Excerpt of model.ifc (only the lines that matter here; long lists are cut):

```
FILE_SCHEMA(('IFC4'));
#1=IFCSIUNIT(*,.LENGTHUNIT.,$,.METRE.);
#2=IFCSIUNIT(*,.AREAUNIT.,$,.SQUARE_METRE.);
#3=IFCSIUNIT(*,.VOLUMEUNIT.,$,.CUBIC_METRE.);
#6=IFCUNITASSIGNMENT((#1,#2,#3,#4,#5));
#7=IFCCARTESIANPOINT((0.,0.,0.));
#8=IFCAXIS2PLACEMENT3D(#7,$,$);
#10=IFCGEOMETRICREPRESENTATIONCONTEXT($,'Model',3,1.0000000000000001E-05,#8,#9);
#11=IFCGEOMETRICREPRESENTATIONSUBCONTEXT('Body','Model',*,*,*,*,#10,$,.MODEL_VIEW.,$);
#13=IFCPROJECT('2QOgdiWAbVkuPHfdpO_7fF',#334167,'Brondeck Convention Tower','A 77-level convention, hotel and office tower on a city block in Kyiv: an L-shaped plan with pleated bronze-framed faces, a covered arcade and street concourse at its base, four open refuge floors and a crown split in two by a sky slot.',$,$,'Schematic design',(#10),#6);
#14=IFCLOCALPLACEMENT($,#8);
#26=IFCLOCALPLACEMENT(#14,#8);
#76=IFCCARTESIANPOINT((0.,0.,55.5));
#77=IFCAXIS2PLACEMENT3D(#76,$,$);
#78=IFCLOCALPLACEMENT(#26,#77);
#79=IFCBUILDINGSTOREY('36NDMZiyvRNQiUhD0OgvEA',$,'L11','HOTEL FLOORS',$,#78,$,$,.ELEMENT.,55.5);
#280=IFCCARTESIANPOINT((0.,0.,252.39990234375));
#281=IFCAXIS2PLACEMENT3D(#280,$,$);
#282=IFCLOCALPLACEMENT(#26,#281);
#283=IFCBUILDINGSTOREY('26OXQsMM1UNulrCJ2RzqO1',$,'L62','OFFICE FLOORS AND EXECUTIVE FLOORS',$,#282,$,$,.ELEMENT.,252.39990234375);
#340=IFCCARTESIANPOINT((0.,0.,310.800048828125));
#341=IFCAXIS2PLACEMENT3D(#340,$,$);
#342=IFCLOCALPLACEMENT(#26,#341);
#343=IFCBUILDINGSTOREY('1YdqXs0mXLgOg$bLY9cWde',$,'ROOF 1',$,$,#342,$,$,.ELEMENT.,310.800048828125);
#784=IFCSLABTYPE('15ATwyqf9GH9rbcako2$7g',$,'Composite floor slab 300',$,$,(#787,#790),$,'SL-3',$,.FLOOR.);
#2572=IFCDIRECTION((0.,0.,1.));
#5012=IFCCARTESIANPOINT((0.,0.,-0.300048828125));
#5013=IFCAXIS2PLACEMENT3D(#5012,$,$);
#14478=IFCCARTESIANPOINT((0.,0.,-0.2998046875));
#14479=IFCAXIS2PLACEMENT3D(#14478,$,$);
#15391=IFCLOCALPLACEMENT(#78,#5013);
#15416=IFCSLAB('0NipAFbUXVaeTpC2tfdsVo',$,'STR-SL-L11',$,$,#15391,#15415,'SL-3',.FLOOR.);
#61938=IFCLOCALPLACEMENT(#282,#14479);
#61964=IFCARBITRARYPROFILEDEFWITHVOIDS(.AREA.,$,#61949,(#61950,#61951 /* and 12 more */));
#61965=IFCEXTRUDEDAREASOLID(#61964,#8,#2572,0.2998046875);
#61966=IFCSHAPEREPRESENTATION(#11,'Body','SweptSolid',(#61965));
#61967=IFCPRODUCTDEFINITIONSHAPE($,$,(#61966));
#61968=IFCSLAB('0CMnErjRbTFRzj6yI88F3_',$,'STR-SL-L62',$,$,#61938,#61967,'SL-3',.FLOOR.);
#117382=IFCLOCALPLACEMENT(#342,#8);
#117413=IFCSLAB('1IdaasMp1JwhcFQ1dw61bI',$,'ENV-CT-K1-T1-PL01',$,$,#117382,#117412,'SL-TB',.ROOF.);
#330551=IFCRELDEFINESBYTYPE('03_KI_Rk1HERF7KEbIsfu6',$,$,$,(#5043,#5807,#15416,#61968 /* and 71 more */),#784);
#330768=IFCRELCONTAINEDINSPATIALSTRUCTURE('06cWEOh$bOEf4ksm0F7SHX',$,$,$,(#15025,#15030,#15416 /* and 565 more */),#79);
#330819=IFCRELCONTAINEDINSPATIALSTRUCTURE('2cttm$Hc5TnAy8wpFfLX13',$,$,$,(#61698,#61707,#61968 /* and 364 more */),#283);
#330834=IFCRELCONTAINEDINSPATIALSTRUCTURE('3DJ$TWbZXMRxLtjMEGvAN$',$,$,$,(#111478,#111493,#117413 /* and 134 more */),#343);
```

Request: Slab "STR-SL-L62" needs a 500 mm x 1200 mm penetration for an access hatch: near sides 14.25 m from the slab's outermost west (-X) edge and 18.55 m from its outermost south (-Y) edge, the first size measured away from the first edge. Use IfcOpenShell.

```python
import numpy as np
import ifcopenshell
import ifcopenshell.api.feature
import ifcopenshell.api.geometry
import ifcopenshell.api.root
import ifcopenshell.geom
import ifcopenshell.util.placement
import ifcopenshell.util.representation
import ifcopenshell.util.shape
import ifcopenshell.util.unit

model = ifcopenshell.open("model.ifc")
unit_scale = ifcopenshell.util.unit.calculate_unit_scale(model)
settings = ifcopenshell.geom.settings()


def volume(element):
    """Net volume in cubic metres, openings subtracted."""
    shape = ifcopenshell.geom.create_shape(settings, element)
    return ifcopenshell.util.shape.get_volume(shape.geometry)


slab = model.by_guid("0CMnErjRbTFRzj6yI88F3_")
before = volume(slab)

# Extent in the slab's own axes, in metres. The edges named are its -X and -Y sides.
slab_shape = ifcopenshell.geom.create_shape(settings, slab)
vertices = ifcopenshell.util.shape.get_vertices(slab_shape.geometry)
x_min, y_min, bottom = vertices.min(axis=0)
top = vertices[:, 2].max()

opening = ifcopenshell.api.root.create_entity(model, ifc_class="IfcOpeningElement", name="Access hatch opening", predefined_type="OPENING")
context = ifcopenshell.util.representation.get_context(model, "Model", "Body", "MODEL_VIEW")
width, depth = 0.5, 1.2
outline = [(0.0, 0.0), (width, 0.0), (width, depth), (0.0, depth), (0.0, 0.0)]
# Overshoot both faces by 50 mm so the cut is clean.
shape = ifcopenshell.api.geometry.add_slab_representation(
    model, context=context, depth=top - bottom + 0.1, polyline=outline
)
ifcopenshell.api.geometry.assign_representation(model, product=opening, representation=shape)

matrix = ifcopenshell.util.placement.get_local_placement(slab.ObjectPlacement)
matrix[:, 3] = matrix @ np.append(np.array([x_min + 14.25, y_min + 18.55, bottom - 0.05]) / unit_scale, 1.0)
ifcopenshell.api.geometry.edit_object_placement(model, product=opening, matrix=matrix, is_si=False)
ifcopenshell.api.feature.add_feature(model, feature=opening, element=slab)

after = volume(slab)

print(f"slab volume {before:.3f} -> {after:.3f} m3")

model.write("model-out.ifc")
```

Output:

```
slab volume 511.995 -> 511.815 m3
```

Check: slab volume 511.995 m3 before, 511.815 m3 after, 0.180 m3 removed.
